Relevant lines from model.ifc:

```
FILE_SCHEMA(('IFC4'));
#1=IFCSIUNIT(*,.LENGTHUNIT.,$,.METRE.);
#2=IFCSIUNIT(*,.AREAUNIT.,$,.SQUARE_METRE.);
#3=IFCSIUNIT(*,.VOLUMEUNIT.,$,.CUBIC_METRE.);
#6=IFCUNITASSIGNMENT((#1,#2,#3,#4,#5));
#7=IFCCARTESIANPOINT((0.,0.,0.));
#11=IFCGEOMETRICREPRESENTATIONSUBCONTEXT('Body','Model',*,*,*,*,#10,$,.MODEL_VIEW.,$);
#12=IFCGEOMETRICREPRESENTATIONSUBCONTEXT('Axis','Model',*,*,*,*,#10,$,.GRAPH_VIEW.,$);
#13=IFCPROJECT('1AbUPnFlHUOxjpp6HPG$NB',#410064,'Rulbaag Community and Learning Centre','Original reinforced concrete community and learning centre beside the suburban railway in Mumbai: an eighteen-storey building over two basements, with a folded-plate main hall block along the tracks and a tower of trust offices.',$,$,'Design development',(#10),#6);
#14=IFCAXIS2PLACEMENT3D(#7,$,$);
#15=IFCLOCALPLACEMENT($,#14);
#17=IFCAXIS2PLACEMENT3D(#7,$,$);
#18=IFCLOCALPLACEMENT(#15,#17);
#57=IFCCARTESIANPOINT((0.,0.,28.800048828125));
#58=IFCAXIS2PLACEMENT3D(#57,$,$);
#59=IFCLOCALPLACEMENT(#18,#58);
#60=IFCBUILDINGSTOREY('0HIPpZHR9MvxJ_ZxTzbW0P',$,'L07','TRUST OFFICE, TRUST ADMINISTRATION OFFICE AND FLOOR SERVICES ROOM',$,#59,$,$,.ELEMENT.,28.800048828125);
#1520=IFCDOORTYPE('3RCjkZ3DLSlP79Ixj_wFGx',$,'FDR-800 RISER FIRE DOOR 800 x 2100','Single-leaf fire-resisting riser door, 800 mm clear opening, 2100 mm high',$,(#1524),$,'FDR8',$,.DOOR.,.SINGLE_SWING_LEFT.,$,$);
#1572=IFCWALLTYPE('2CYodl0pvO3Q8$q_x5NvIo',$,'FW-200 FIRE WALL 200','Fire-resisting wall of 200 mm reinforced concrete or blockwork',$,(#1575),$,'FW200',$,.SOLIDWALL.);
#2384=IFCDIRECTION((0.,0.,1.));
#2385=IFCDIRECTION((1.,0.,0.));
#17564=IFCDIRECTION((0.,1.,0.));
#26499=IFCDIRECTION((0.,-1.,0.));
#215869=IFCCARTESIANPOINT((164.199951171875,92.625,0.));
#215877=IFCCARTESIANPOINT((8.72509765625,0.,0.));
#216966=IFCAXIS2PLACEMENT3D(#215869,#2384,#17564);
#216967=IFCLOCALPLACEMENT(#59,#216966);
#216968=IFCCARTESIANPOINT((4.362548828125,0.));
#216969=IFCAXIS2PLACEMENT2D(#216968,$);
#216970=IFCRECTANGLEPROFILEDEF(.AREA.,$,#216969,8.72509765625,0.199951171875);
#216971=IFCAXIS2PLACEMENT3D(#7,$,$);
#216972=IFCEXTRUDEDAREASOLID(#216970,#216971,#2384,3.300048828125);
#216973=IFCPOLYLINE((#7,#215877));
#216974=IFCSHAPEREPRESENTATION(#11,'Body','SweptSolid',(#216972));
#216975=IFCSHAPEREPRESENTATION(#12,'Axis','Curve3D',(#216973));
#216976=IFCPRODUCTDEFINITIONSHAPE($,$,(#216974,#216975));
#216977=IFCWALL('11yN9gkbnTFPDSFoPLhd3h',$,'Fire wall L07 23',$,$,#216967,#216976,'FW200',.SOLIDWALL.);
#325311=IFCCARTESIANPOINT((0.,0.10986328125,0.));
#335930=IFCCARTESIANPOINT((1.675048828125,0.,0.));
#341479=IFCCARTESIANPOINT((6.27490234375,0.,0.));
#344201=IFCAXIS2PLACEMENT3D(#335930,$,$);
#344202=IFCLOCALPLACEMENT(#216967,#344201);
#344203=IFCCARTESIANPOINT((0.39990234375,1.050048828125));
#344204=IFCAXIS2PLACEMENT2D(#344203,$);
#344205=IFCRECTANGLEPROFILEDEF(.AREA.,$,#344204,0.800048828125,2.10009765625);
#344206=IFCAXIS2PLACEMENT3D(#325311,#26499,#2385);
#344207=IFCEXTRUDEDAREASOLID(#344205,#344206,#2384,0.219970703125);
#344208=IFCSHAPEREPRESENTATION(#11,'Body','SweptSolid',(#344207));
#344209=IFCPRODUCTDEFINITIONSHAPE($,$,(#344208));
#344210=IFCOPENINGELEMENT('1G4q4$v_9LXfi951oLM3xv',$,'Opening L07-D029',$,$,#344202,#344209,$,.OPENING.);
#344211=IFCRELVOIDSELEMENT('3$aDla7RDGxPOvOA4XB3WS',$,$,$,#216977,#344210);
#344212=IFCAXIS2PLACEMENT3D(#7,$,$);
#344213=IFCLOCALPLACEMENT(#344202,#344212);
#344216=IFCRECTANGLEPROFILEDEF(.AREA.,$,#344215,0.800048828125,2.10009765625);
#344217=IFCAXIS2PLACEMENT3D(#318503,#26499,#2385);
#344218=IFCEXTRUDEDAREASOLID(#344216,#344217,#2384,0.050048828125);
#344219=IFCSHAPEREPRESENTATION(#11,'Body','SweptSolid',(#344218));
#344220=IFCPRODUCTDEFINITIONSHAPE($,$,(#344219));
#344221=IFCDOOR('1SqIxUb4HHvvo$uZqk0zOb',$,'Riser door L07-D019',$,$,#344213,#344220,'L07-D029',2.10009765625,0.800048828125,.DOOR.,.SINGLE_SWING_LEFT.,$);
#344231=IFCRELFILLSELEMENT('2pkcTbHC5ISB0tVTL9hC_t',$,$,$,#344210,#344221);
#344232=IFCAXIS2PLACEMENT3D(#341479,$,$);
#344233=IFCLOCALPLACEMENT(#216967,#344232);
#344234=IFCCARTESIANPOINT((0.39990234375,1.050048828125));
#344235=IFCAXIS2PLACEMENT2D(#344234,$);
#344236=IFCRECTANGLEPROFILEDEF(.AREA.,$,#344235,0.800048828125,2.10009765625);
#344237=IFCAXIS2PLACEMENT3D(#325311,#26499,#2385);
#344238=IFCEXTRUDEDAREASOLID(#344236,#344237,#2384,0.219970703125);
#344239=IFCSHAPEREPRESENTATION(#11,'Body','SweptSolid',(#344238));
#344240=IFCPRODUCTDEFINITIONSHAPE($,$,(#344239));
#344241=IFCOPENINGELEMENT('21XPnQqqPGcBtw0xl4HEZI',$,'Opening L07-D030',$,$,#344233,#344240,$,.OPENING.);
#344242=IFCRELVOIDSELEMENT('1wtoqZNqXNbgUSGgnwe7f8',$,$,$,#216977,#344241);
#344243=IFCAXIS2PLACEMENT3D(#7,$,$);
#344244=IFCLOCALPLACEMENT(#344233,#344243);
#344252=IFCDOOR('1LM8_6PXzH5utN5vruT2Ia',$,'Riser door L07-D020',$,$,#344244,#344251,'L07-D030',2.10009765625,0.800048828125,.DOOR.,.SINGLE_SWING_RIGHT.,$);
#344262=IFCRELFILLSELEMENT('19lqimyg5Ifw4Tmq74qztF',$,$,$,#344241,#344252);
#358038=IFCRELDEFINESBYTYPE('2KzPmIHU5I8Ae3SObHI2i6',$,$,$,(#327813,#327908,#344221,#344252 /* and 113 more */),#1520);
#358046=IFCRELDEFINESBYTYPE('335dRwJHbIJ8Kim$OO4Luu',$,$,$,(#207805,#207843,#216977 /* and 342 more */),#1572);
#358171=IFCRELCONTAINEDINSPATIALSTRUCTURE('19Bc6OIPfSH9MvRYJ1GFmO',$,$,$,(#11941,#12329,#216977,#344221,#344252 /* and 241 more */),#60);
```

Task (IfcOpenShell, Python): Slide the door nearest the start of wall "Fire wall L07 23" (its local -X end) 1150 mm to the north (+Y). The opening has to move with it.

```python
import ifcopenshell
import ifcopenshell.api.geometry
import ifcopenshell.util.placement

model = ifcopenshell.open("model.ifc")

door = model.by_id(344221)
opening = door.FillsVoids[0].RelatingOpeningElement
wall = opening.VoidsElements[0].RelatingBuildingElement

wall_matrix = ifcopenshell.util.placement.get_local_placement(wall.ObjectPlacement)
shift = wall_matrix[:3, 0] * 1.15
before = ifcopenshell.util.placement.get_local_placement(door.ObjectPlacement)[:3, 3].copy()

# The door is placed relative to its opening, so it follows when the opening moves.
matrix = ifcopenshell.util.placement.get_local_placement(opening.ObjectPlacement)
matrix[:3, 3] += shift
ifcopenshell.api.geometry.edit_object_placement(
    model, product=opening, matrix=matrix, is_si=False, should_transform_children=True
)

after = ifcopenshell.util.placement.get_local_placement(door.ObjectPlacement)[:3, 3]
print("door moved by", (after - before).round(3) + 0.0)

model.write("model_rev.ifc")
```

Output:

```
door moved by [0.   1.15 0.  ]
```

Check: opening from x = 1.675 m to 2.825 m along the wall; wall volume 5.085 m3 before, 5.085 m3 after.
